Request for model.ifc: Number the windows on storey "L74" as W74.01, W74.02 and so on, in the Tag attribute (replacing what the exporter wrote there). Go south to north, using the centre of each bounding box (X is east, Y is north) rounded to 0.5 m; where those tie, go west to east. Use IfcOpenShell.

First a look at what the model holds.

```python
import ifcopenshell
import ifcopenshell.util.element
import ifcopenshell.util.placement

model = ifcopenshell.open("model.ifc")
print(model.schema)
storey = next(s for s in model.by_type("IfcBuildingStorey") if s.Name == "L74")
windows = [e for e in ifcopenshell.util.element.get_decomposition(storey) if e.is_a("IfcWindow")]
for e in sorted(windows, key=lambda e: e.id()):
    origin = ifcopenshell.util.placement.get_local_placement(e.ObjectPlacement)[:3, 3]
    print(e.id(), e.Tag, e.Name, origin.round(2) + 0.0, sep=" | ")
```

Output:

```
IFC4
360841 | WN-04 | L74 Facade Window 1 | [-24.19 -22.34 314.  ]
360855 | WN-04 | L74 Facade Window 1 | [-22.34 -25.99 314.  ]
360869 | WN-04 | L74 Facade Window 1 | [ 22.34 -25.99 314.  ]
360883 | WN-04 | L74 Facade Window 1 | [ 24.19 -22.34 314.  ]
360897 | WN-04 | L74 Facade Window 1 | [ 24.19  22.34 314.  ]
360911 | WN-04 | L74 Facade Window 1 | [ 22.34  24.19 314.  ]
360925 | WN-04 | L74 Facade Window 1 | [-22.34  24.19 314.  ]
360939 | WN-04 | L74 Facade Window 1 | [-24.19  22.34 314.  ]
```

```python
import ifcopenshell
import ifcopenshell.geom
import ifcopenshell.util.element
import ifcopenshell.util.shape

model = ifcopenshell.open("model.ifc")
settings = ifcopenshell.geom.settings()
settings.set("use-world-coords", True)


def centre(element):
    shape = ifcopenshell.geom.create_shape(settings, element)
    return ifcopenshell.util.shape.get_bbox_centroid(shape.geometry)


storey = next(s for s in model.by_type("IfcBuildingStorey") if s.Name == "L74")
windows = [e for e in ifcopenshell.util.element.get_decomposition(storey) if e.is_a("IfcWindow")]

# Insertion points can sit at a corner or the storey origin, so sort by the geometry (in metres).
centres = {e: centre(e) for e in windows}
windows.sort(key=lambda e: (round(centres[e][1] / 0.5), centres[e][0]))

for i, e in enumerate(windows, start=1):
    number = f"W74.{i:02d}"
    e.Tag = number
    print(e.id(), number)

model.write("model-out.ifc")
```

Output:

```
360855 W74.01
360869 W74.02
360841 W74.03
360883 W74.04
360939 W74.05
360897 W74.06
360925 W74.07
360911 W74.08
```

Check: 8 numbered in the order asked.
